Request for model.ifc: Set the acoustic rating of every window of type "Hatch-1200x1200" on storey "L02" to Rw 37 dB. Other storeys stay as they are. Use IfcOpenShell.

First a look at what the model holds.

```python
import ifcopenshell
import ifcopenshell.util.element

model = ifcopenshell.open("model.ifc")
print(model.schema)
storey = next(s for s in model.by_type("IfcBuildingStorey") if s.Name == "L02")
windows = [e for e in ifcopenshell.util.element.get_decomposition(storey) if e.is_a("IfcWindow")]
seen = {}
for e in windows:
    element_type = ifcopenshell.util.element.get_type(e)
    key = (element_type.Name if element_type != e and element_type else None, ifcopenshell.util.element.get_pset(e, "Pset_WindowCommon", "AcousticRating"))
    seen[key] = seen.get(key, 0) + 1
for (name, value), count in sorted(seen.items(), key=str):
    print(count, "x", name, "|", value)
```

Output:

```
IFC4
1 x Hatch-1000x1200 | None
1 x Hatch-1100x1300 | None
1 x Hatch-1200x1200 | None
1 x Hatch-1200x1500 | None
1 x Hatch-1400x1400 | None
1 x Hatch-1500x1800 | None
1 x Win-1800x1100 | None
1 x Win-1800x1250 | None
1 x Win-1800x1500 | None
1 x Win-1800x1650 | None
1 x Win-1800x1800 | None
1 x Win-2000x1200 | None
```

```python
import ifcopenshell
import ifcopenshell.api.pset
import ifcopenshell.util.element

model = ifcopenshell.open("model.ifc")

storey = next(s for s in model.by_type("IfcBuildingStorey") if s.Name == "L02")
windows = [e for e in ifcopenshell.util.element.get_decomposition(storey) if e.is_a("IfcWindow")]

count = 0
for e in windows:
    element_type = ifcopenshell.util.element.get_type(e)
    if element_type in (None, e) or element_type.Name != "Hatch-1200x1200":
        continue
    # add_pset returns the element's existing set when there is one.
    pset = ifcopenshell.api.pset.add_pset(model, product=e, name="Pset_WindowCommon")
    ifcopenshell.api.pset.edit_pset(model, pset=pset, properties={"AcousticRating": "Rw 37 dB"})
    count += 1

print(count, "windows updated")

model.write("model_updated.ifc")
```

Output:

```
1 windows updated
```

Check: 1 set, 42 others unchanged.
